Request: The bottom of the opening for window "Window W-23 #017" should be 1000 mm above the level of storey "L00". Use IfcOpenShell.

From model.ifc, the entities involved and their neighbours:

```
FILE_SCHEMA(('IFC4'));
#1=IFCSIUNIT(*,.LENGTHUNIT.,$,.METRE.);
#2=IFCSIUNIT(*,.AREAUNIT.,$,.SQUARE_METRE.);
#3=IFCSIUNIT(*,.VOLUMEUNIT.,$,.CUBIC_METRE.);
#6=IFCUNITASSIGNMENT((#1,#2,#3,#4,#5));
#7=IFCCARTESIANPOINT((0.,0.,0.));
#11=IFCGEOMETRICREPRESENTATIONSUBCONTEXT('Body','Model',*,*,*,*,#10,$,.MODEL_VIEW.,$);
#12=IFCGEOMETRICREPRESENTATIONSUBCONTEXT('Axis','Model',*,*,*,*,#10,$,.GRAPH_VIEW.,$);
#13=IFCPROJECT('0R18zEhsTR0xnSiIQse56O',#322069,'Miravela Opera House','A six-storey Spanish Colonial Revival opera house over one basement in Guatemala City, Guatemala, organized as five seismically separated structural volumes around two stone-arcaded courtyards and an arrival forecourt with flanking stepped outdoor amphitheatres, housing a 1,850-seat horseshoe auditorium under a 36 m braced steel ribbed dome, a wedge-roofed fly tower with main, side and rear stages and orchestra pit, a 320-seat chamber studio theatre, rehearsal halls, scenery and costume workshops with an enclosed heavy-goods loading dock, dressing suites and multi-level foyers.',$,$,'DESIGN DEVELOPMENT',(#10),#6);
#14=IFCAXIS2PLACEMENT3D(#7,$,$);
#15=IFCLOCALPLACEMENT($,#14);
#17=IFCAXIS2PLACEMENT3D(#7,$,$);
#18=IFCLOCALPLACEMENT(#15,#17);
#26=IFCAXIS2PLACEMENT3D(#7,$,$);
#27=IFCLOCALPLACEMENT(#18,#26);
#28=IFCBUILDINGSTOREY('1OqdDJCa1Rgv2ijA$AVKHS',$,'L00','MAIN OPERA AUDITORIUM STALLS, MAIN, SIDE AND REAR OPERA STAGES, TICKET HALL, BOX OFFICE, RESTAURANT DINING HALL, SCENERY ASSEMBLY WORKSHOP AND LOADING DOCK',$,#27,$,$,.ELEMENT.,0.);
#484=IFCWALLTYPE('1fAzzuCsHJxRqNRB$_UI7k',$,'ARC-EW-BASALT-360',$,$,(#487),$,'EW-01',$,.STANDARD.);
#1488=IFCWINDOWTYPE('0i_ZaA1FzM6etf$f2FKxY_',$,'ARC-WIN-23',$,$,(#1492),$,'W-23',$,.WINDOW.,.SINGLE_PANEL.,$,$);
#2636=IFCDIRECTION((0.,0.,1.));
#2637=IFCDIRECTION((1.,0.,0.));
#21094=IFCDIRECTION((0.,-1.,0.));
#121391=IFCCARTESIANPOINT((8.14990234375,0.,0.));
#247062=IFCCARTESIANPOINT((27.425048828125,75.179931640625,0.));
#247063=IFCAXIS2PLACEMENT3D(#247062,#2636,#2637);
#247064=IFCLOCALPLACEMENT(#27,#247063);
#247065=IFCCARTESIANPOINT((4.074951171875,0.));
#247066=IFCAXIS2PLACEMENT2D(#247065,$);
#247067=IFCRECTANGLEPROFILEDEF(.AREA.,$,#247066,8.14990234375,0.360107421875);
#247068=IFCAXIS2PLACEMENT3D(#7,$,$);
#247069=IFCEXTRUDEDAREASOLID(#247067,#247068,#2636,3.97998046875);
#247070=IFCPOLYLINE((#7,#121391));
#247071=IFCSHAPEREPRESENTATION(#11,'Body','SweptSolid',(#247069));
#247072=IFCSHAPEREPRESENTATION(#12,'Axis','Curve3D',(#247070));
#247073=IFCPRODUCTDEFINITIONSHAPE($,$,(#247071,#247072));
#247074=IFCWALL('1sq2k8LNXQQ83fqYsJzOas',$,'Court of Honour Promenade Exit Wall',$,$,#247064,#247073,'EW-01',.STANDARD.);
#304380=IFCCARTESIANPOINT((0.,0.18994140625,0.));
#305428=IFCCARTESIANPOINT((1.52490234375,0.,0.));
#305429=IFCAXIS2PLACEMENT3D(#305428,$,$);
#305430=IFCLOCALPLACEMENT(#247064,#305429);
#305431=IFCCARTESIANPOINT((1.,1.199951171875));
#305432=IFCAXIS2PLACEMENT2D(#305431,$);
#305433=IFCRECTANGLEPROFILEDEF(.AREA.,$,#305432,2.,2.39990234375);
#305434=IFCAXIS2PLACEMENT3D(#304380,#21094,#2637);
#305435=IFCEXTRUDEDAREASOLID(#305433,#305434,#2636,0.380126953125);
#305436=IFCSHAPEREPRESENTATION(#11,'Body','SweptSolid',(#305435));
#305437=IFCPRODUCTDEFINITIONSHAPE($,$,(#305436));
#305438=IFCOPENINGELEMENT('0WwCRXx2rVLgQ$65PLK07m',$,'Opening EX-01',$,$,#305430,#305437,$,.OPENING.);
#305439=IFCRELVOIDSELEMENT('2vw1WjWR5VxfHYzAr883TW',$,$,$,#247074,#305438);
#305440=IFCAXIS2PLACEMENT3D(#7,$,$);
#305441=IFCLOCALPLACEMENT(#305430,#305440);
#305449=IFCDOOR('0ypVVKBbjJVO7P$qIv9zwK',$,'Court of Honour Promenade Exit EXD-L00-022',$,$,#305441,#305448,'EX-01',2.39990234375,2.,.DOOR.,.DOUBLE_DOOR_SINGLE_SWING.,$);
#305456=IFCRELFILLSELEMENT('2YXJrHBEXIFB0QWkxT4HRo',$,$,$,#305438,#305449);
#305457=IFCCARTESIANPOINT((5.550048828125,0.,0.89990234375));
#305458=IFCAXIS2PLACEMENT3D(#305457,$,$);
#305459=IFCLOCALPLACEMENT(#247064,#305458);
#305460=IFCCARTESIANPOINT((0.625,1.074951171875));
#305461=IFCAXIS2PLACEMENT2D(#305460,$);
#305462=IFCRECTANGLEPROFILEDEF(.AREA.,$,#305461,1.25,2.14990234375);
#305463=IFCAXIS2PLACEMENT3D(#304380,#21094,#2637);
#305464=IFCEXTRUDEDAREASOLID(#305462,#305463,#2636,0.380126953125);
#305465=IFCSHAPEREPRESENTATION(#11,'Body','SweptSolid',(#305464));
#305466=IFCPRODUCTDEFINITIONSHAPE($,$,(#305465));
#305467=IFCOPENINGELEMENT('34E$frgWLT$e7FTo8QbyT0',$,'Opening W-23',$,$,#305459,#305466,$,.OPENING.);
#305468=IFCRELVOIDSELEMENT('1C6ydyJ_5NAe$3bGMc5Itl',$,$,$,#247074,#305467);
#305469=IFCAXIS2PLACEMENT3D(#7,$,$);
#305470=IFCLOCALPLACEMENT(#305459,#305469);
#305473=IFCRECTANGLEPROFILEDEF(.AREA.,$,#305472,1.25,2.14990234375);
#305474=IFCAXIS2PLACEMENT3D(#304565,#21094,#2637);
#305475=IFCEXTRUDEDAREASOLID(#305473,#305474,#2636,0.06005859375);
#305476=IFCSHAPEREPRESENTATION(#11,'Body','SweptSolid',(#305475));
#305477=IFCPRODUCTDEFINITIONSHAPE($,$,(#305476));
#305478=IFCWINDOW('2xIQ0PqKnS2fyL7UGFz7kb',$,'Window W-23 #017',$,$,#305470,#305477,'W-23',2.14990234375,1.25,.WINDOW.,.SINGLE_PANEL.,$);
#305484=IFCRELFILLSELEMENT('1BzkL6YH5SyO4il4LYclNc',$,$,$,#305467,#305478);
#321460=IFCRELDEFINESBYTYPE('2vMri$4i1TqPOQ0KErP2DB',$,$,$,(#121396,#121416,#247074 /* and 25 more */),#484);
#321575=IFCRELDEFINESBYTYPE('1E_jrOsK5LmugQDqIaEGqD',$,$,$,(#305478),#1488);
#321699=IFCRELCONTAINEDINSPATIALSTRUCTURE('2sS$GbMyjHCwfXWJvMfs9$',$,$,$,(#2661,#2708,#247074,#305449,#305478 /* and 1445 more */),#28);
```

```python
import numpy as np
import ifcopenshell
import ifcopenshell.api.geometry
import ifcopenshell.geom
import ifcopenshell.util.element
import ifcopenshell.util.placement
import ifcopenshell.util.shape
import ifcopenshell.util.unit

model = ifcopenshell.open("model.ifc")
unit_scale = ifcopenshell.util.unit.calculate_unit_scale(model)

window = model.by_guid("2xIQ0PqKnS2fyL7UGFz7kb")
opening = window.FillsVoids[0].RelatingOpeningElement
storey = ifcopenshell.util.element.get_container(window, ifc_class="IfcBuildingStorey")
level = ifcopenshell.util.placement.get_local_placement(storey.ObjectPlacement)[2, 3]

# The opening's origin need not be at the sill, so measure its lowest point.
shape = ifcopenshell.geom.create_shape(ifcopenshell.geom.settings(), opening)
bottom = ifcopenshell.util.shape.get_shape_bottom_elevation(shape, shape.geometry) / unit_scale
dz = level + 1 / unit_scale - bottom

shift = np.array([0.0, 0.0, dz])
# The window is placed relative to its opening, so it follows when the opening moves.
matrix = ifcopenshell.util.placement.get_local_placement(opening.ObjectPlacement)
matrix[:3, 3] += shift
ifcopenshell.api.geometry.edit_object_placement(
    model, product=opening, matrix=matrix, is_si=False, should_transform_children=True
)

print(f"moved by {dz * unit_scale:+.3f} m")

model.write("model_edited.ifc")
```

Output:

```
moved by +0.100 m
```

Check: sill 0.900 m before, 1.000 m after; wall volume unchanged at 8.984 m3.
